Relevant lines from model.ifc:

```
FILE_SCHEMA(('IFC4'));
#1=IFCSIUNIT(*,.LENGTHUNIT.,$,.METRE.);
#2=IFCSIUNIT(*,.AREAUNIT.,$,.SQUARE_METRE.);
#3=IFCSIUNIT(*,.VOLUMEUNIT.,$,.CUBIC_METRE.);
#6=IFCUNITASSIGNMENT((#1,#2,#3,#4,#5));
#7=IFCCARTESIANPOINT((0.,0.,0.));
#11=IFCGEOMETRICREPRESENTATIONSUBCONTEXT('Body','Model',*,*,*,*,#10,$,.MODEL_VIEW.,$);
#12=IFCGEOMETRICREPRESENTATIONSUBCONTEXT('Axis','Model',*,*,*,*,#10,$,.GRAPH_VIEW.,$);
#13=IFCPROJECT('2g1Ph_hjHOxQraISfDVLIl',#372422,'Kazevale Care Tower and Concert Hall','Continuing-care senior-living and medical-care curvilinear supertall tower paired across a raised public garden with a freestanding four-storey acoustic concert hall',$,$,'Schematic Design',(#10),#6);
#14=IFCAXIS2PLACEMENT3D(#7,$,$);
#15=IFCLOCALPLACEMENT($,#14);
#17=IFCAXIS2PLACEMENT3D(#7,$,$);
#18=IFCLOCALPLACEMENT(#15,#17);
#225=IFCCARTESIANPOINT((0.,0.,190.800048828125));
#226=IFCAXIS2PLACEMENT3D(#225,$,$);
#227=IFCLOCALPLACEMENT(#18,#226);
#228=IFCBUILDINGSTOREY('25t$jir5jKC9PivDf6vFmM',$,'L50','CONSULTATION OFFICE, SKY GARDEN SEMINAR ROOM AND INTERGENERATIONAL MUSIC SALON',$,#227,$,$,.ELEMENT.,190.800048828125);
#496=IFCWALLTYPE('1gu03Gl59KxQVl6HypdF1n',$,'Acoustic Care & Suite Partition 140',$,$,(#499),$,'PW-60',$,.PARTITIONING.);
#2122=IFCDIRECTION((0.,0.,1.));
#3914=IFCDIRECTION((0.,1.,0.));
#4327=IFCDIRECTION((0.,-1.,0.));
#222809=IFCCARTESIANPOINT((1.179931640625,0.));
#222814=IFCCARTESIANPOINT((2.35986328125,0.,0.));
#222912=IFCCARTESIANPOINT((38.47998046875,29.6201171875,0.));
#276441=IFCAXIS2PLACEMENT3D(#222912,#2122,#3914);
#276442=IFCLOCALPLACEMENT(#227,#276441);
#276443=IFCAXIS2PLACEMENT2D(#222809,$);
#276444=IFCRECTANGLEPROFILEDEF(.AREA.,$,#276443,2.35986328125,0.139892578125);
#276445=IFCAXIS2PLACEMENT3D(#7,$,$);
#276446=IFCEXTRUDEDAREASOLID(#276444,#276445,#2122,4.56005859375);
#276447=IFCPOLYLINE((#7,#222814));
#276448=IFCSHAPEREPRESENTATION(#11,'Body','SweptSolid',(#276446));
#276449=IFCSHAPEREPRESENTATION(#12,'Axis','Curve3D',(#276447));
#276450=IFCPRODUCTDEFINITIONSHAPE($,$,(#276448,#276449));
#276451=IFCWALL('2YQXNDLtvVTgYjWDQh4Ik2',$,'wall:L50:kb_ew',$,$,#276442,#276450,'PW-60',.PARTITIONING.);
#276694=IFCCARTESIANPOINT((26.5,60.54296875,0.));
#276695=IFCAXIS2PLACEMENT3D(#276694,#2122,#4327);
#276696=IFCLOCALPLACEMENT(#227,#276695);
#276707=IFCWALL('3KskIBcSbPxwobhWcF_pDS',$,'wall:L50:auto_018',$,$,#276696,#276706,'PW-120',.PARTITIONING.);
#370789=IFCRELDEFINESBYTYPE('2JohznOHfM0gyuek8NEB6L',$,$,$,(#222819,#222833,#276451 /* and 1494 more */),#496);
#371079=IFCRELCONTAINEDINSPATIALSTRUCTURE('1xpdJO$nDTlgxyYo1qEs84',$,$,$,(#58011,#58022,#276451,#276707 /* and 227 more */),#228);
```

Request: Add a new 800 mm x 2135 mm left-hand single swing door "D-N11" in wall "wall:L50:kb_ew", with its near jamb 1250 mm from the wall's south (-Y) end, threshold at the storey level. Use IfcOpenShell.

```python
import numpy as np
import ifcopenshell
import ifcopenshell.api.feature
import ifcopenshell.api.geometry
import ifcopenshell.api.root
import ifcopenshell.api.spatial
import ifcopenshell.geom
import ifcopenshell.util.element
import ifcopenshell.util.placement
import ifcopenshell.util.representation
import ifcopenshell.util.shape
import ifcopenshell.util.unit

model = ifcopenshell.open("model.ifc")
unit_scale = ifcopenshell.util.unit.calculate_unit_scale(model)
settings = ifcopenshell.geom.settings()


def volume(element):
    """Net volume in cubic metres, openings subtracted."""
    shape = ifcopenshell.geom.create_shape(settings, element)
    return ifcopenshell.util.shape.get_volume(shape.geometry)


wall = model.by_id(276451)
storey = ifcopenshell.util.element.get_container(wall, ifc_class="IfcBuildingStorey")
context = ifcopenshell.util.representation.get_context(model, "Model", "Body", "MODEL_VIEW")
before = volume(wall)

width, height, from_end, sill = 0.8, 2.135, 1.25, 0.0  # metres

# The wall runs along its own X axis, and the end named is its -X end.
wall_shape = ifcopenshell.geom.create_shape(settings, wall)
x, y, z = ifcopenshell.util.shape.get_vertices(wall_shape.geometry).T
start = x.min() + from_end
face, thickness = float(y.min()), float(y.max() - y.min())
wall_matrix = ifcopenshell.util.placement.get_local_placement(wall.ObjectPlacement)
level = ifcopenshell.util.placement.get_local_placement(storey.ObjectPlacement)[2, 3]


def in_wall(x, y):
    """Placement at x, y metres in the wall's axes, at sill height."""
    matrix = wall_matrix.copy()
    matrix[:, 3] = wall_matrix @ np.array([x / unit_scale, y / unit_scale, 0.0, 1.0])
    matrix[2, 3] = level + sill / unit_scale
    return matrix


# Opening: a box that overshoots both wall faces by 50 mm.
opening = ifcopenshell.api.root.create_entity(model, ifc_class="IfcOpeningElement", predefined_type="OPENING")
box = ifcopenshell.api.geometry.add_wall_representation(
    model, context=context, length=width, height=height, thickness=thickness + 0.1
)
ifcopenshell.api.geometry.assign_representation(model, product=opening, representation=box)
ifcopenshell.api.geometry.edit_object_placement(model, product=opening, matrix=in_wall(start, face - 0.05), is_si=False)
ifcopenshell.api.feature.add_feature(model, feature=opening, element=wall)

door = ifcopenshell.api.root.create_entity(model, ifc_class="IfcDoor", name="D-N11", predefined_type="DOOR")
door.OverallWidth, door.OverallHeight = width / unit_scale, height / unit_scale
door.OperationType = "SINGLE_SWING_LEFT"
body = ifcopenshell.api.geometry.add_door_representation(
    model,
    context=context,
    overall_width=door.OverallWidth,
    overall_height=door.OverallHeight,
    operation_type="SINGLE_SWING_LEFT",
    lining_properties={"LiningDepth": thickness / unit_scale, "ThresholdDepth": thickness / unit_scale},
)
ifcopenshell.api.geometry.assign_representation(model, product=door, representation=body)
ifcopenshell.api.spatial.assign_container(model, products=[door], relating_structure=storey)
ifcopenshell.api.feature.add_filling(model, opening=opening, element=door)

# The lining spans the wall, so the door starts at the wall face.
ifcopenshell.api.geometry.edit_object_placement(model, product=door, matrix=in_wall(start, face), is_si=False)

after = volume(wall)

print(f"wall volume {before:.3f} -> {after:.3f} m3")

model.write("model-out.ifc")
```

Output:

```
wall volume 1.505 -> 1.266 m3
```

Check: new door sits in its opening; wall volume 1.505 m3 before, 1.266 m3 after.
